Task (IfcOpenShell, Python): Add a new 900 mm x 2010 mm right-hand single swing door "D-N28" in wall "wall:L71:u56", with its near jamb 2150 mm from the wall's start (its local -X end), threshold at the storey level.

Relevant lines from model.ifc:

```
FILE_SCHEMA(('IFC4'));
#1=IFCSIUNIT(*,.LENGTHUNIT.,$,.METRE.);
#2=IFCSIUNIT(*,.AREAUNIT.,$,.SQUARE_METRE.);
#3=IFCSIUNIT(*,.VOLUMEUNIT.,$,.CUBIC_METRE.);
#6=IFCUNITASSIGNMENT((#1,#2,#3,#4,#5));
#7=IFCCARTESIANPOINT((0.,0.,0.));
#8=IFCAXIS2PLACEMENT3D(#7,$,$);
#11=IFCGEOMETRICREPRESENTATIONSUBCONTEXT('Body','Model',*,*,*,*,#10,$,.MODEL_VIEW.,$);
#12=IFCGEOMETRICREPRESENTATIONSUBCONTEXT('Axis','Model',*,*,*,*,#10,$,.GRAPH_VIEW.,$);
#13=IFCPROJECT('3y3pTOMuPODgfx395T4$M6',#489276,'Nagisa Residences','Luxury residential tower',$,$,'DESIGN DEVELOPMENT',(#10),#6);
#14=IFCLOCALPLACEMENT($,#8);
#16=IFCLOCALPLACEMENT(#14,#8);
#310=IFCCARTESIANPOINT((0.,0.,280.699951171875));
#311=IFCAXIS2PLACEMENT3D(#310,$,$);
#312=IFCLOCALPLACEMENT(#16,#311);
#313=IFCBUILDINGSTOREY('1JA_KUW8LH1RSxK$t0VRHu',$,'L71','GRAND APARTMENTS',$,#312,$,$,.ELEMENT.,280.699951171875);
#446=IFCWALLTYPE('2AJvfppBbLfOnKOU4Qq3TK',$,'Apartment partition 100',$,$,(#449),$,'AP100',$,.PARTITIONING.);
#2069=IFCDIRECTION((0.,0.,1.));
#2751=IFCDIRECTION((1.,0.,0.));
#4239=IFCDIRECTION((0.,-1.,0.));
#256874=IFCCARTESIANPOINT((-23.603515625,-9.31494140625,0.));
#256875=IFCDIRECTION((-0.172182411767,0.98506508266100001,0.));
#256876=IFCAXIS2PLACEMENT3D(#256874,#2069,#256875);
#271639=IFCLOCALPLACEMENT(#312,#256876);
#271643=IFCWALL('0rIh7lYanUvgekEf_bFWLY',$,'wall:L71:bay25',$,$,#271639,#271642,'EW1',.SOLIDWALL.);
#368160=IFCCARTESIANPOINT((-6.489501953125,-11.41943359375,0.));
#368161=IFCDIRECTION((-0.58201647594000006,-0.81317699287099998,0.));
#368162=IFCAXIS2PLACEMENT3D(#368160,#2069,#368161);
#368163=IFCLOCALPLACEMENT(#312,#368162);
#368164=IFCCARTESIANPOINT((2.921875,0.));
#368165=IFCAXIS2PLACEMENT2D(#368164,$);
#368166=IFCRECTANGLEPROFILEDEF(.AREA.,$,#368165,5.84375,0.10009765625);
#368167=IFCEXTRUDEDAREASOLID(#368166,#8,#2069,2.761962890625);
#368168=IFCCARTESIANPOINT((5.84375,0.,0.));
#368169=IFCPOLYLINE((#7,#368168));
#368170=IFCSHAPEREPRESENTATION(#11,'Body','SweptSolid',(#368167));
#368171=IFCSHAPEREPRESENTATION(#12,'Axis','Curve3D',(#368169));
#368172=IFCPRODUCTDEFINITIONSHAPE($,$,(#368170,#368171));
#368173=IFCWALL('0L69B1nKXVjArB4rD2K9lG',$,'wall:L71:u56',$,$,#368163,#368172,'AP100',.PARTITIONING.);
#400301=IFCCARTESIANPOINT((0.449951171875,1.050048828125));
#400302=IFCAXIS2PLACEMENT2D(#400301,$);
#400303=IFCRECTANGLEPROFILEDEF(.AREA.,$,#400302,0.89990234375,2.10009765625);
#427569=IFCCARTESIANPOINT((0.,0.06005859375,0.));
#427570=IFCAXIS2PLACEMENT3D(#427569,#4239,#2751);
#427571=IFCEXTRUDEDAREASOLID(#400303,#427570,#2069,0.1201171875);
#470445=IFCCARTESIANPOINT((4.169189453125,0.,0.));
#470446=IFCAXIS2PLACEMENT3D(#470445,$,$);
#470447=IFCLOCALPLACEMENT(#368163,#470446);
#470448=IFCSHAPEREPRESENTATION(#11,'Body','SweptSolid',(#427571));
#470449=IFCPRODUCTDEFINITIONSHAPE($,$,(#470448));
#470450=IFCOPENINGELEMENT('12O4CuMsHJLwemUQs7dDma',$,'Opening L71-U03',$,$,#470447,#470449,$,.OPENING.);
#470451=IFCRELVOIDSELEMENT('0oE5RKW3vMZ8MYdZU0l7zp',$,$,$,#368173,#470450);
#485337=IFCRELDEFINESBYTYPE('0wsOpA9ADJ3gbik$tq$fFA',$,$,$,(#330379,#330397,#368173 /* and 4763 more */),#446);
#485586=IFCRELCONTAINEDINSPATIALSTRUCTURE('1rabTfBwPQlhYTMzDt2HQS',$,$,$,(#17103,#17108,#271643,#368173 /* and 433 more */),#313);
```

```python
import numpy as np
import ifcopenshell
import ifcopenshell.api.feature
import ifcopenshell.api.geometry
import ifcopenshell.api.root
import ifcopenshell.api.spatial
import ifcopenshell.geom
import ifcopenshell.util.element
import ifcopenshell.util.placement
import ifcopenshell.util.representation
import ifcopenshell.util.shape
import ifcopenshell.util.unit

model = ifcopenshell.open("model.ifc")
unit_scale = ifcopenshell.util.unit.calculate_unit_scale(model)
settings = ifcopenshell.geom.settings()


def volume(element):
    """Net volume in cubic metres, openings subtracted."""
    shape = ifcopenshell.geom.create_shape(settings, element)
    return ifcopenshell.util.shape.get_volume(shape.geometry)


wall = model.by_id(368173)
storey = ifcopenshell.util.element.get_container(wall, ifc_class="IfcBuildingStorey")
context = ifcopenshell.util.representation.get_context(model, "Model", "Body", "MODEL_VIEW")
before = volume(wall)

width, height, from_end, sill = 0.9, 2.01, 2.15, 0.0  # metres

# The wall runs along its own X axis, and the end named is its -X end.
wall_shape = ifcopenshell.geom.create_shape(settings, wall)
x, y, z = ifcopenshell.util.shape.get_vertices(wall_shape.geometry).T
start = x.min() + from_end
face, thickness = float(y.min()), float(y.max() - y.min())
wall_matrix = ifcopenshell.util.placement.get_local_placement(wall.ObjectPlacement)
level = ifcopenshell.util.placement.get_local_placement(storey.ObjectPlacement)[2, 3]


def in_wall(x, y):
    """Placement at x, y metres in the wall's axes, at sill height."""
    matrix = wall_matrix.copy()
    matrix[:, 3] = wall_matrix @ np.array([x / unit_scale, y / unit_scale, 0.0, 1.0])
    matrix[2, 3] = level + sill / unit_scale
    return matrix


# Opening: a box that overshoots both wall faces by 50 mm.
opening = ifcopenshell.api.root.create_entity(model, ifc_class="IfcOpeningElement", predefined_type="OPENING")
box = ifcopenshell.api.geometry.add_wall_representation(
    model, context=context, length=width, height=height, thickness=thickness + 0.1
)
ifcopenshell.api.geometry.assign_representation(model, product=opening, representation=box)
ifcopenshell.api.geometry.edit_object_placement(model, product=opening, matrix=in_wall(start, face - 0.05), is_si=False)
ifcopenshell.api.feature.add_feature(model, feature=opening, element=wall)

door = ifcopenshell.api.root.create_entity(model, ifc_class="IfcDoor", name="D-N28", predefined_type="DOOR")
door.OverallWidth, door.OverallHeight = width / unit_scale, height / unit_scale
door.OperationType = "SINGLE_SWING_RIGHT"
body = ifcopenshell.api.geometry.add_door_representation(
    model,
    context=context,
    overall_width=door.OverallWidth,
    overall_height=door.OverallHeight,
    operation_type="SINGLE_SWING_RIGHT",
    lining_properties={"LiningDepth": thickness / unit_scale, "ThresholdDepth": thickness / unit_scale},
)
ifcopenshell.api.geometry.assign_representation(model, product=door, representation=body)
ifcopenshell.api.spatial.assign_container(model, products=[door], relating_structure=storey)
ifcopenshell.api.feature.add_filling(model, opening=opening, element=door)

# The lining spans the wall, so the door starts at the wall face.
ifcopenshell.api.geometry.edit_object_placement(model, product=door, matrix=in_wall(start, face), is_si=False)

after = volume(wall)

print(f"wall volume {before:.3f} -> {after:.3f} m3")

model.write("model-out.ifc")
```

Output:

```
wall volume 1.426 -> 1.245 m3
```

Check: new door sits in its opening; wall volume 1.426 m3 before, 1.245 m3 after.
